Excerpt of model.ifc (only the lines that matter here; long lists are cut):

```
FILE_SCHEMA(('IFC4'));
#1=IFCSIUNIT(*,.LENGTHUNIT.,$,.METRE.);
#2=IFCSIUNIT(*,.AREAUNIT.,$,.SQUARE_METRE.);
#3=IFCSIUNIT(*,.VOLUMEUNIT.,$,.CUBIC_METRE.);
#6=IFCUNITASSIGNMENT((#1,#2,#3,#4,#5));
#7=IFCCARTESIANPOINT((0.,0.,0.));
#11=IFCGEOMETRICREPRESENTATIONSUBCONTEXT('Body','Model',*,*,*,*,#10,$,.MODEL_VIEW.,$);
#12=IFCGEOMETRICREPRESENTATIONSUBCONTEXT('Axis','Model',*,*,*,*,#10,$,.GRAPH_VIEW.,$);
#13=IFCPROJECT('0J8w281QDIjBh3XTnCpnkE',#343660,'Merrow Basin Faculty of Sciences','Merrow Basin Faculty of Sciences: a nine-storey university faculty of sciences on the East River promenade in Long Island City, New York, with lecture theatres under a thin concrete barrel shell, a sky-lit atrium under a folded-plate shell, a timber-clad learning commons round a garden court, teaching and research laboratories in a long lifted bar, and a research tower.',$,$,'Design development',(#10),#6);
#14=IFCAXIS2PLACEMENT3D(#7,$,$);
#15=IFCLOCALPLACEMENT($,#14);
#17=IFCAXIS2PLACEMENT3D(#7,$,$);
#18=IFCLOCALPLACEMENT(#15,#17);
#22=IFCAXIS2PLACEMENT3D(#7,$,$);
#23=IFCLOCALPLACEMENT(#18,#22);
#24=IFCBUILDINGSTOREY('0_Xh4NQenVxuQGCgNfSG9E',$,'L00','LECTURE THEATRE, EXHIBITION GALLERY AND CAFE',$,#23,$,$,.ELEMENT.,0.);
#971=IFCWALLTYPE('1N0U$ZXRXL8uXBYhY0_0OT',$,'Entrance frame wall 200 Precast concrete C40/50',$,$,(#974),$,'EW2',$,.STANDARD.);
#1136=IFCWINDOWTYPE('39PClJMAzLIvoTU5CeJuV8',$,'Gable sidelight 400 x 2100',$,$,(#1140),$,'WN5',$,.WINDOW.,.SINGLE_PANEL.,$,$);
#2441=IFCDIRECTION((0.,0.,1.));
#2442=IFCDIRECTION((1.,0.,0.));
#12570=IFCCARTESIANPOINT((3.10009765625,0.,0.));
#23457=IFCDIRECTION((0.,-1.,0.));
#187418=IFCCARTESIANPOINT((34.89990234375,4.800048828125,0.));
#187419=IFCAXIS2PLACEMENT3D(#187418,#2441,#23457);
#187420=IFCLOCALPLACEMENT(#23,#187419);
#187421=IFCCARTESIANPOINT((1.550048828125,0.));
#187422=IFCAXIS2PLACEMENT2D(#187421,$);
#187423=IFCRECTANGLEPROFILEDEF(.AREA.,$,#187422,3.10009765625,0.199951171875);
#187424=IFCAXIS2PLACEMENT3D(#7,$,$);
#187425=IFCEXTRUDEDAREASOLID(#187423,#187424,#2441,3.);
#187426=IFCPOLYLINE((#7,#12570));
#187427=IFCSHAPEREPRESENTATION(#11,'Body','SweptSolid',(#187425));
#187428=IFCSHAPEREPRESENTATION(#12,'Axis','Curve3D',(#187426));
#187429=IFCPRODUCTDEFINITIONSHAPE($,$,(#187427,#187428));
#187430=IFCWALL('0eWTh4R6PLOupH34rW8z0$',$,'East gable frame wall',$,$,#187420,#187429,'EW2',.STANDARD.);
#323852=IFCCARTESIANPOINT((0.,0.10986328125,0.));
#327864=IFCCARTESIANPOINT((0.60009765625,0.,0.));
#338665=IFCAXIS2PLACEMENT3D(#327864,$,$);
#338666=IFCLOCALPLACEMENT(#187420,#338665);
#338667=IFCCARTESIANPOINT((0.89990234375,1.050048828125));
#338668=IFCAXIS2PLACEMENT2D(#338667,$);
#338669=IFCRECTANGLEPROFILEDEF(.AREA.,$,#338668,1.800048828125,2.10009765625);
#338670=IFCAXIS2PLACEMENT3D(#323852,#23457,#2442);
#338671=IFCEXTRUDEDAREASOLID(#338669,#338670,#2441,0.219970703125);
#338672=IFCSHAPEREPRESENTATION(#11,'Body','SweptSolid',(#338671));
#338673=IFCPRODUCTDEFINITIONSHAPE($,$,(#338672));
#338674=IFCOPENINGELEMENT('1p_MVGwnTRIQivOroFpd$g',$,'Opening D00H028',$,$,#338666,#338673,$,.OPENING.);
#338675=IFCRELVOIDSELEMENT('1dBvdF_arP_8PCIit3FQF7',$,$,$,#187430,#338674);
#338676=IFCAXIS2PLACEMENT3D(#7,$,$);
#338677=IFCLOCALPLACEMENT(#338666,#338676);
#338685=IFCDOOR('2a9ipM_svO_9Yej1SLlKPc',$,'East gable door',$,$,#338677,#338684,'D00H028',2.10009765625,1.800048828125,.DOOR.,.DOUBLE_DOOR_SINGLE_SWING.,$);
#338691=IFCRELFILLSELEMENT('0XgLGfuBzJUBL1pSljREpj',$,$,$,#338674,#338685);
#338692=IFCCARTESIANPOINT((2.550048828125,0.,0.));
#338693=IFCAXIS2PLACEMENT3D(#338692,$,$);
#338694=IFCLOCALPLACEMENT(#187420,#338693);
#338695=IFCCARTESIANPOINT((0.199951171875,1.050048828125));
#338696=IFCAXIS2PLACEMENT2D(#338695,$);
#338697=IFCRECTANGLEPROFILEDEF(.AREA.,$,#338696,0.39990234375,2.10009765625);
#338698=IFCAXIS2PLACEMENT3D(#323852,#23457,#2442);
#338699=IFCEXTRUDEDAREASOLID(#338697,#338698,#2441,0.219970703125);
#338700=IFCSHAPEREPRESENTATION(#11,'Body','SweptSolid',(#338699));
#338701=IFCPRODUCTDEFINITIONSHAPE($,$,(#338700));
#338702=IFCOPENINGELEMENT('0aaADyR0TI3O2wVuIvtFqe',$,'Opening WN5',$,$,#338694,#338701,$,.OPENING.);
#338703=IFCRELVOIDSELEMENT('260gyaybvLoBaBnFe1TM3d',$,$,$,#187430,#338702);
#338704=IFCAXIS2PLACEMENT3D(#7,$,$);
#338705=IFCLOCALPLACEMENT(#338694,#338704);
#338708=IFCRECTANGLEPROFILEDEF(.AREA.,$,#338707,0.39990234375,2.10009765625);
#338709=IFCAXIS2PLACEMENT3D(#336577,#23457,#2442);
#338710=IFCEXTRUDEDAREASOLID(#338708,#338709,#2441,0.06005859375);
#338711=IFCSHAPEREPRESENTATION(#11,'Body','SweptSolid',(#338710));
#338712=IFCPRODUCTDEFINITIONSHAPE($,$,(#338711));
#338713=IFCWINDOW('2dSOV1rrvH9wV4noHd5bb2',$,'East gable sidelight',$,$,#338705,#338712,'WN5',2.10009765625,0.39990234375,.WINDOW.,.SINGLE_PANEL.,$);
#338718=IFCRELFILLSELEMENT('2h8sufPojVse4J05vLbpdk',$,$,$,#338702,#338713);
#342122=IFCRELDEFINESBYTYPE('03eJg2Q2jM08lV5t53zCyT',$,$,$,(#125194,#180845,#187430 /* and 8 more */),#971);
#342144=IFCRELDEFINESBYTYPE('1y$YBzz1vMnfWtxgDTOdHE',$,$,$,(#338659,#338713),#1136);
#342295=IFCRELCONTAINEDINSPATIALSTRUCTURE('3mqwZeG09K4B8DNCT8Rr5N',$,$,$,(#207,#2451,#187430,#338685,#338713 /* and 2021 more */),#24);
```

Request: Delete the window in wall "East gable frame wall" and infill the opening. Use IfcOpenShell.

```python
import ifcopenshell
import ifcopenshell.api.feature
import ifcopenshell.api.root
import ifcopenshell.geom
import ifcopenshell.util.shape

model = ifcopenshell.open("model.ifc")
settings = ifcopenshell.geom.settings()


def volume(element):
    """Net volume in cubic metres, openings subtracted."""
    shape = ifcopenshell.geom.create_shape(settings, element)
    return ifcopenshell.util.shape.get_volume(shape.geometry)


window = model.by_guid("2dSOV1rrvH9wV4noHd5bb2")
opening = window.FillsVoids[0].RelatingOpeningElement
wall = opening.VoidsElements[0].RelatingBuildingElement
before = volume(wall)

ifcopenshell.api.root.remove_product(model, product=window)
ifcopenshell.api.feature.remove_feature(model, feature=opening)

after = volume(wall)

print(f"wall volume {before:.3f} -> {after:.3f} m3")

model.write("model_edited.ifc")
```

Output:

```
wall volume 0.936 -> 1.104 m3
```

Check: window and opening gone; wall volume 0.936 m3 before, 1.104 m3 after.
